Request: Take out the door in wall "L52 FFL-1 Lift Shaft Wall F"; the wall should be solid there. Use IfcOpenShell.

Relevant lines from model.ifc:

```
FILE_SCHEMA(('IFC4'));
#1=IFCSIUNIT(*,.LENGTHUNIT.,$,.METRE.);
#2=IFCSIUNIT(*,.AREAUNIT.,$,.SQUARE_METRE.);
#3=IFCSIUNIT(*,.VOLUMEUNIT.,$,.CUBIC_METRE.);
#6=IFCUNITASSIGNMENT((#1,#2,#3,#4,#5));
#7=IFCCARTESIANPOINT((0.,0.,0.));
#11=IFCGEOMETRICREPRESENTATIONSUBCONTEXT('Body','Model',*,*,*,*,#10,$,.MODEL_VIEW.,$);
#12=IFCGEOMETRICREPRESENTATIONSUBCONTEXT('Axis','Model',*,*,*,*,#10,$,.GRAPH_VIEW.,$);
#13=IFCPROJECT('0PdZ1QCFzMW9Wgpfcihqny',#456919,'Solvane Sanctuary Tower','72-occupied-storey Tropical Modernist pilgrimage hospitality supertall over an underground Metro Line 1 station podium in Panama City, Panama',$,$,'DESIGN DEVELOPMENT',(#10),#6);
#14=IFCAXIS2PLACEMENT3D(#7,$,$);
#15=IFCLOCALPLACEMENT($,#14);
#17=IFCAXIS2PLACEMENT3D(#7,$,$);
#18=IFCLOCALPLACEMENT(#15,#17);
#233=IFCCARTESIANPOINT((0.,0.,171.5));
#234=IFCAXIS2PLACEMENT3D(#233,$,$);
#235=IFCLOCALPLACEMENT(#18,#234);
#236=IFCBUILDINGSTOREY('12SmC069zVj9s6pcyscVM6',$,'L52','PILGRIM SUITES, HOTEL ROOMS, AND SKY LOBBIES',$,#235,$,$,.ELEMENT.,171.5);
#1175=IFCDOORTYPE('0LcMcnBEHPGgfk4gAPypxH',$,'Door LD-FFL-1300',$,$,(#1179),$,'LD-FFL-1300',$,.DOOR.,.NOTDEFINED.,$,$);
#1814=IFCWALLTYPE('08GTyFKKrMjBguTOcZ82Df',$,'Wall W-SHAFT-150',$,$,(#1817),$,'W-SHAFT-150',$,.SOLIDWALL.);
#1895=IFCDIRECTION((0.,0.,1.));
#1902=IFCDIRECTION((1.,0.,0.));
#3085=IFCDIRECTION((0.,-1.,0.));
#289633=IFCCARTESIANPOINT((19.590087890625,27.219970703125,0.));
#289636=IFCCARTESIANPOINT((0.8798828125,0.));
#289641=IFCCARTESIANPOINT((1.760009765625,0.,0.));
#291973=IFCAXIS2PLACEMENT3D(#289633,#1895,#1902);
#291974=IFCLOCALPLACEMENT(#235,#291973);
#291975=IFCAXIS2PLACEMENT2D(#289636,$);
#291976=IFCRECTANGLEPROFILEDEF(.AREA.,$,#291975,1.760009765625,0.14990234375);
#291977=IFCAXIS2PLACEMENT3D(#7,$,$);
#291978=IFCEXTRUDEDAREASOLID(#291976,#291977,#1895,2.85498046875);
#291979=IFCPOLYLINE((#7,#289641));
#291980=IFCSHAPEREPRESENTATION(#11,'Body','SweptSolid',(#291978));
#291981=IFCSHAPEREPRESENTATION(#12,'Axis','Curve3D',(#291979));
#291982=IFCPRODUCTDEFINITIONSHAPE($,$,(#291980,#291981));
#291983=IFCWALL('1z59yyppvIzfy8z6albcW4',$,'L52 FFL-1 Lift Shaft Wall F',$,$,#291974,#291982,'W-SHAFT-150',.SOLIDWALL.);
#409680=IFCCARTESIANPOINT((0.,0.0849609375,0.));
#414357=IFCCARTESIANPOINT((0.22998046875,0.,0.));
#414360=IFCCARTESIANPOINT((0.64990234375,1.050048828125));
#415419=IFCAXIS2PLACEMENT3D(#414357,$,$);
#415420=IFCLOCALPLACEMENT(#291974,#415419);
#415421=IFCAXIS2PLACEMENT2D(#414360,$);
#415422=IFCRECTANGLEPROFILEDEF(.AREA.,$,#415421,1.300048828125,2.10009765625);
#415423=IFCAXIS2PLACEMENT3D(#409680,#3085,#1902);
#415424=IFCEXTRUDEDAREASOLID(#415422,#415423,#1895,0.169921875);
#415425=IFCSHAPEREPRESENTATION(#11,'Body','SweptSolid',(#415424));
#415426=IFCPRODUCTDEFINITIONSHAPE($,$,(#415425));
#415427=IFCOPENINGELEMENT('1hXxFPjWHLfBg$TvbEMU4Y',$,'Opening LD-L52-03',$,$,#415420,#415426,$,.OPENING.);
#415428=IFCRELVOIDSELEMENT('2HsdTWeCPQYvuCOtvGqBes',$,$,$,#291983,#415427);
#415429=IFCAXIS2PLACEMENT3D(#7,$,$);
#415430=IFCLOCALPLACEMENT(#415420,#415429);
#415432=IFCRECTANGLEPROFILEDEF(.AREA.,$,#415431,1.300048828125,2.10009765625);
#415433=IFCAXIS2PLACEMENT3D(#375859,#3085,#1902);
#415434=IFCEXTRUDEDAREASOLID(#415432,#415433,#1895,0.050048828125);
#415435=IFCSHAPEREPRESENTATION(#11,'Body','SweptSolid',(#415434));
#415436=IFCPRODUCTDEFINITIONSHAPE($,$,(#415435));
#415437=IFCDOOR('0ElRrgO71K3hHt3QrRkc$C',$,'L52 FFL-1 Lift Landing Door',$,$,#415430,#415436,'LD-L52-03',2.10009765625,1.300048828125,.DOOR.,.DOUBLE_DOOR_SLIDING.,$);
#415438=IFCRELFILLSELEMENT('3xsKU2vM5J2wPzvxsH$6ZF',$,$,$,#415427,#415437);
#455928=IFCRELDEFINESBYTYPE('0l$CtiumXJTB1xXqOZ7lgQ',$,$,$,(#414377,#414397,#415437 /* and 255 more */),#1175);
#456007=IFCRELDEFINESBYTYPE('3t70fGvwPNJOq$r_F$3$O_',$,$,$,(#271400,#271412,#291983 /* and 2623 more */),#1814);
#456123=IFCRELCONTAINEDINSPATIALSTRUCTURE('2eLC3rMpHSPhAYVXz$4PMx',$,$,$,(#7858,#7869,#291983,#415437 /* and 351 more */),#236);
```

```python
import ifcopenshell
import ifcopenshell.api.feature
import ifcopenshell.api.root
import ifcopenshell.geom
import ifcopenshell.util.shape

model = ifcopenshell.open("model.ifc")
settings = ifcopenshell.geom.settings()


def volume(element):
    """Net volume in cubic metres, openings subtracted."""
    shape = ifcopenshell.geom.create_shape(settings, element)
    return ifcopenshell.util.shape.get_volume(shape.geometry)


door = model.by_guid("0ElRrgO71K3hHt3QrRkc$C")
opening = door.FillsVoids[0].RelatingOpeningElement
wall = opening.VoidsElements[0].RelatingBuildingElement
before = volume(wall)

ifcopenshell.api.root.remove_product(model, product=door)
ifcopenshell.api.feature.remove_feature(model, feature=opening)

after = volume(wall)

print(f"wall volume {before:.3f} -> {after:.3f} m3")

model.write("model_v2.ifc")
```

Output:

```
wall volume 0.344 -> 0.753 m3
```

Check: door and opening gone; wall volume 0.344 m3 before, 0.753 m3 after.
